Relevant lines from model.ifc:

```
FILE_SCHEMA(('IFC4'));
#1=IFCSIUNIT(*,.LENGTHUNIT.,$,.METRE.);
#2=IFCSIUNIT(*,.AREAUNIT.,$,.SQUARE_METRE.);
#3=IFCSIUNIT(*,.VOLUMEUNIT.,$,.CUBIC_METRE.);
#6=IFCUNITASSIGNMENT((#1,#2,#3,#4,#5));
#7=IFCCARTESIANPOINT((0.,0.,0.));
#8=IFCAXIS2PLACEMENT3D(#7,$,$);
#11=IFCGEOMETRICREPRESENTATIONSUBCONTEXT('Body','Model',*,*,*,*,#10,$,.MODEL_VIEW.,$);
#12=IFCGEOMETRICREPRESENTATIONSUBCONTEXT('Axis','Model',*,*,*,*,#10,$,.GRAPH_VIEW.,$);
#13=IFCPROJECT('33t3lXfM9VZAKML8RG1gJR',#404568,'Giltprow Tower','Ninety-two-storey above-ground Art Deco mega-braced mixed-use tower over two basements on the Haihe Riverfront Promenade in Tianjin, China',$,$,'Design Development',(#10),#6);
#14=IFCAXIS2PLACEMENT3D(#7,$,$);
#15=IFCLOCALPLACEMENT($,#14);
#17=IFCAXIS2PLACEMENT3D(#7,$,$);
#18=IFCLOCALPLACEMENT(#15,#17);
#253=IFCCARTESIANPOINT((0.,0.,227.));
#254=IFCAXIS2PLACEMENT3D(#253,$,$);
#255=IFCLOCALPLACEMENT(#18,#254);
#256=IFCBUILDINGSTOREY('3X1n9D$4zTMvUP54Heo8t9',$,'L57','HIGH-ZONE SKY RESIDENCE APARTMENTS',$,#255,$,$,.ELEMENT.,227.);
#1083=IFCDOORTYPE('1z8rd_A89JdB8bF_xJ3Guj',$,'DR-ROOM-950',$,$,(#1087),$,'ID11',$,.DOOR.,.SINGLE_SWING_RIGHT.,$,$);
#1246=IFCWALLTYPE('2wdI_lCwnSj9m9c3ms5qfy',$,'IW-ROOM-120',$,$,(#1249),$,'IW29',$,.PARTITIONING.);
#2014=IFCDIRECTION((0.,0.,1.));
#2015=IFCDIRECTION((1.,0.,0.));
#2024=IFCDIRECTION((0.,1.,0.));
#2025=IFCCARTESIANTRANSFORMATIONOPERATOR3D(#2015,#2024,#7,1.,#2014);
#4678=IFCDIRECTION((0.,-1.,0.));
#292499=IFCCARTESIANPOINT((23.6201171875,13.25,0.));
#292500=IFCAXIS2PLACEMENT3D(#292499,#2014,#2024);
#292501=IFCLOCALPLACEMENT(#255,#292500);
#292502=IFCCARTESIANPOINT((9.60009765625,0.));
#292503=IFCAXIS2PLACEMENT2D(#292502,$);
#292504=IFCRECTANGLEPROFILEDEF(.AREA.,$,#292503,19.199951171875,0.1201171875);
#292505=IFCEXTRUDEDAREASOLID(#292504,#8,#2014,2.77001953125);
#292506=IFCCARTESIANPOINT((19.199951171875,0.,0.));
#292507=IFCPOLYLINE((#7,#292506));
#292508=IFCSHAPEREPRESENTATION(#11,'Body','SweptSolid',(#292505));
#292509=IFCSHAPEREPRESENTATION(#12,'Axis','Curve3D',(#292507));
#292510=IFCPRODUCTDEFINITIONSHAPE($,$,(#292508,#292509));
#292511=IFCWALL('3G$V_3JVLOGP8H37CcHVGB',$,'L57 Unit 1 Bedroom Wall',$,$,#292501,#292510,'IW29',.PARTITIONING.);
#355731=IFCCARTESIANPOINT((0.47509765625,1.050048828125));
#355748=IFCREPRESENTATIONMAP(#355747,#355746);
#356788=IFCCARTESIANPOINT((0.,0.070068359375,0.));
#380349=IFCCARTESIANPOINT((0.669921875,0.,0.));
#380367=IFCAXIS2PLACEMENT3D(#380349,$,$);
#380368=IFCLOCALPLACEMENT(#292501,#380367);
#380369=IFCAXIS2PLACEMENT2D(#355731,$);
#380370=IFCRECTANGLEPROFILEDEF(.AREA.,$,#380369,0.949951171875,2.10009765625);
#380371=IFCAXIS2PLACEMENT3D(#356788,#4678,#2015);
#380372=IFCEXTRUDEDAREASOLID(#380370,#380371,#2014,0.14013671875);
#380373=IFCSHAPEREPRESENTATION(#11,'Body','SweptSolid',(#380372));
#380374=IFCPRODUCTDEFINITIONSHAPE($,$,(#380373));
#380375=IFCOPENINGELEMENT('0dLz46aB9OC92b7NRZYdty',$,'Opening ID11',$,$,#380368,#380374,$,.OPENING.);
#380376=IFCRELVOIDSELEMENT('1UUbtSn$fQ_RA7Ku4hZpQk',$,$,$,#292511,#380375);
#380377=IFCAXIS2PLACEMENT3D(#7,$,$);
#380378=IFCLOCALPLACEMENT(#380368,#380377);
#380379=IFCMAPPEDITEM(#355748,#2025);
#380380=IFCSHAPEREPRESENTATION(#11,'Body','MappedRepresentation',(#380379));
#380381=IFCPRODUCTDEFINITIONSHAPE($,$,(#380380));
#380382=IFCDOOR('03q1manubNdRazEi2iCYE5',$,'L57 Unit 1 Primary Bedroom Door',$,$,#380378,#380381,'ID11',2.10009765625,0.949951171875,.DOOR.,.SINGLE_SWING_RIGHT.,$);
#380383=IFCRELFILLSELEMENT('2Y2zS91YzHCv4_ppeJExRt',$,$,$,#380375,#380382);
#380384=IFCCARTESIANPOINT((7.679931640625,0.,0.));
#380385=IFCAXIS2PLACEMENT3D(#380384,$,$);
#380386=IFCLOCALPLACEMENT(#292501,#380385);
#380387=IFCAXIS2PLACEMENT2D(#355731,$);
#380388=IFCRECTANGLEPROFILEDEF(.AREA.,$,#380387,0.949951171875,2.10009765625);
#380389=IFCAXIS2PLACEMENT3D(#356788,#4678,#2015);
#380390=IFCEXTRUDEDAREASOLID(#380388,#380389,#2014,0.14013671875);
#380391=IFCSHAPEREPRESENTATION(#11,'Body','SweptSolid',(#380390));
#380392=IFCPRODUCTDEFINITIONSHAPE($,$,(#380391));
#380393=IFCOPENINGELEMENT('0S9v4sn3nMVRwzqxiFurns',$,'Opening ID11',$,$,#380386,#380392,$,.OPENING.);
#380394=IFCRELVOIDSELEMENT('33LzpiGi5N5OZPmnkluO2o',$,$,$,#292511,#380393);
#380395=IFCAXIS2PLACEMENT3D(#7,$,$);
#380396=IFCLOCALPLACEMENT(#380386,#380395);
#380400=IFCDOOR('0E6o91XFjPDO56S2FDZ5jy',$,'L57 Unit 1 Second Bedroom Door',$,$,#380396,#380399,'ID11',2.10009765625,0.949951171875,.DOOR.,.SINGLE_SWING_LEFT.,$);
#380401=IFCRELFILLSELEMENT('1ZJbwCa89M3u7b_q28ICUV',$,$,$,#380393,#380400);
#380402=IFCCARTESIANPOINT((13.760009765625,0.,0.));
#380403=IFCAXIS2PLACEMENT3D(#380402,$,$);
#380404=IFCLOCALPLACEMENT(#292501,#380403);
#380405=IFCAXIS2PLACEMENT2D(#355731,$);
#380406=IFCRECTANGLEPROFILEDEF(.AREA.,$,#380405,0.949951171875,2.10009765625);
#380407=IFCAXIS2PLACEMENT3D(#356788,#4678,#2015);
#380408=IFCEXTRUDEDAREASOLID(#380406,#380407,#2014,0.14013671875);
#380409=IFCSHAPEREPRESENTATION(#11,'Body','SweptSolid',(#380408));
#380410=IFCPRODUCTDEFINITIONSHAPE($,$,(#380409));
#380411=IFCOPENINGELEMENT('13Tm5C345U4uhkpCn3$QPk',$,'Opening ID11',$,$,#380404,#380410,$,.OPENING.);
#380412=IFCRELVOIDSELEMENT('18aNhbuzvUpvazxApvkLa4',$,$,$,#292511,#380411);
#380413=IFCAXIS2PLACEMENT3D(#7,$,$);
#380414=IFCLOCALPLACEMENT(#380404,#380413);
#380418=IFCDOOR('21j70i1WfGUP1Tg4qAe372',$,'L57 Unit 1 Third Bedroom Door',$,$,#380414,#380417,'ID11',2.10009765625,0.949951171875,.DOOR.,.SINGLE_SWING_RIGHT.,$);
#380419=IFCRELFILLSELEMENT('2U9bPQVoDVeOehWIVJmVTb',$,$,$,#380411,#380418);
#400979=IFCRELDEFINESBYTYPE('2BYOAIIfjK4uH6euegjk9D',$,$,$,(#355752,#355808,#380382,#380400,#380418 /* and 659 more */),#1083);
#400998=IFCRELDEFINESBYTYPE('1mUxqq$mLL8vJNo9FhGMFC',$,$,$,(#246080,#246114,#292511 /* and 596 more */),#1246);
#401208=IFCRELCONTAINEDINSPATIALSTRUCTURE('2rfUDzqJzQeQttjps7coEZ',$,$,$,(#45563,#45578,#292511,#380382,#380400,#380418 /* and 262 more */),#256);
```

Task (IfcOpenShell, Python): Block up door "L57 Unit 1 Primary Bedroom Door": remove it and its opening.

```python
import ifcopenshell
import ifcopenshell.api.feature
import ifcopenshell.api.root
import ifcopenshell.geom
import ifcopenshell.util.shape

model = ifcopenshell.open("model.ifc")
settings = ifcopenshell.geom.settings()


def volume(element):
    """Net volume in cubic metres, openings subtracted."""
    shape = ifcopenshell.geom.create_shape(settings, element)
    return ifcopenshell.util.shape.get_volume(shape.geometry)


door = model.by_id(380382)
opening = door.FillsVoids[0].RelatingOpeningElement
wall = opening.VoidsElements[0].RelatingBuildingElement
before = volume(wall)

ifcopenshell.api.root.remove_product(model, product=door)
ifcopenshell.api.feature.remove_feature(model, feature=opening)

after = volume(wall)

print(f"wall volume {before:.3f} -> {after:.3f} m3")

model.write("model_v2.ifc")
```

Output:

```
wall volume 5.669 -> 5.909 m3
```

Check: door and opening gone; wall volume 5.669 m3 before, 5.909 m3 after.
